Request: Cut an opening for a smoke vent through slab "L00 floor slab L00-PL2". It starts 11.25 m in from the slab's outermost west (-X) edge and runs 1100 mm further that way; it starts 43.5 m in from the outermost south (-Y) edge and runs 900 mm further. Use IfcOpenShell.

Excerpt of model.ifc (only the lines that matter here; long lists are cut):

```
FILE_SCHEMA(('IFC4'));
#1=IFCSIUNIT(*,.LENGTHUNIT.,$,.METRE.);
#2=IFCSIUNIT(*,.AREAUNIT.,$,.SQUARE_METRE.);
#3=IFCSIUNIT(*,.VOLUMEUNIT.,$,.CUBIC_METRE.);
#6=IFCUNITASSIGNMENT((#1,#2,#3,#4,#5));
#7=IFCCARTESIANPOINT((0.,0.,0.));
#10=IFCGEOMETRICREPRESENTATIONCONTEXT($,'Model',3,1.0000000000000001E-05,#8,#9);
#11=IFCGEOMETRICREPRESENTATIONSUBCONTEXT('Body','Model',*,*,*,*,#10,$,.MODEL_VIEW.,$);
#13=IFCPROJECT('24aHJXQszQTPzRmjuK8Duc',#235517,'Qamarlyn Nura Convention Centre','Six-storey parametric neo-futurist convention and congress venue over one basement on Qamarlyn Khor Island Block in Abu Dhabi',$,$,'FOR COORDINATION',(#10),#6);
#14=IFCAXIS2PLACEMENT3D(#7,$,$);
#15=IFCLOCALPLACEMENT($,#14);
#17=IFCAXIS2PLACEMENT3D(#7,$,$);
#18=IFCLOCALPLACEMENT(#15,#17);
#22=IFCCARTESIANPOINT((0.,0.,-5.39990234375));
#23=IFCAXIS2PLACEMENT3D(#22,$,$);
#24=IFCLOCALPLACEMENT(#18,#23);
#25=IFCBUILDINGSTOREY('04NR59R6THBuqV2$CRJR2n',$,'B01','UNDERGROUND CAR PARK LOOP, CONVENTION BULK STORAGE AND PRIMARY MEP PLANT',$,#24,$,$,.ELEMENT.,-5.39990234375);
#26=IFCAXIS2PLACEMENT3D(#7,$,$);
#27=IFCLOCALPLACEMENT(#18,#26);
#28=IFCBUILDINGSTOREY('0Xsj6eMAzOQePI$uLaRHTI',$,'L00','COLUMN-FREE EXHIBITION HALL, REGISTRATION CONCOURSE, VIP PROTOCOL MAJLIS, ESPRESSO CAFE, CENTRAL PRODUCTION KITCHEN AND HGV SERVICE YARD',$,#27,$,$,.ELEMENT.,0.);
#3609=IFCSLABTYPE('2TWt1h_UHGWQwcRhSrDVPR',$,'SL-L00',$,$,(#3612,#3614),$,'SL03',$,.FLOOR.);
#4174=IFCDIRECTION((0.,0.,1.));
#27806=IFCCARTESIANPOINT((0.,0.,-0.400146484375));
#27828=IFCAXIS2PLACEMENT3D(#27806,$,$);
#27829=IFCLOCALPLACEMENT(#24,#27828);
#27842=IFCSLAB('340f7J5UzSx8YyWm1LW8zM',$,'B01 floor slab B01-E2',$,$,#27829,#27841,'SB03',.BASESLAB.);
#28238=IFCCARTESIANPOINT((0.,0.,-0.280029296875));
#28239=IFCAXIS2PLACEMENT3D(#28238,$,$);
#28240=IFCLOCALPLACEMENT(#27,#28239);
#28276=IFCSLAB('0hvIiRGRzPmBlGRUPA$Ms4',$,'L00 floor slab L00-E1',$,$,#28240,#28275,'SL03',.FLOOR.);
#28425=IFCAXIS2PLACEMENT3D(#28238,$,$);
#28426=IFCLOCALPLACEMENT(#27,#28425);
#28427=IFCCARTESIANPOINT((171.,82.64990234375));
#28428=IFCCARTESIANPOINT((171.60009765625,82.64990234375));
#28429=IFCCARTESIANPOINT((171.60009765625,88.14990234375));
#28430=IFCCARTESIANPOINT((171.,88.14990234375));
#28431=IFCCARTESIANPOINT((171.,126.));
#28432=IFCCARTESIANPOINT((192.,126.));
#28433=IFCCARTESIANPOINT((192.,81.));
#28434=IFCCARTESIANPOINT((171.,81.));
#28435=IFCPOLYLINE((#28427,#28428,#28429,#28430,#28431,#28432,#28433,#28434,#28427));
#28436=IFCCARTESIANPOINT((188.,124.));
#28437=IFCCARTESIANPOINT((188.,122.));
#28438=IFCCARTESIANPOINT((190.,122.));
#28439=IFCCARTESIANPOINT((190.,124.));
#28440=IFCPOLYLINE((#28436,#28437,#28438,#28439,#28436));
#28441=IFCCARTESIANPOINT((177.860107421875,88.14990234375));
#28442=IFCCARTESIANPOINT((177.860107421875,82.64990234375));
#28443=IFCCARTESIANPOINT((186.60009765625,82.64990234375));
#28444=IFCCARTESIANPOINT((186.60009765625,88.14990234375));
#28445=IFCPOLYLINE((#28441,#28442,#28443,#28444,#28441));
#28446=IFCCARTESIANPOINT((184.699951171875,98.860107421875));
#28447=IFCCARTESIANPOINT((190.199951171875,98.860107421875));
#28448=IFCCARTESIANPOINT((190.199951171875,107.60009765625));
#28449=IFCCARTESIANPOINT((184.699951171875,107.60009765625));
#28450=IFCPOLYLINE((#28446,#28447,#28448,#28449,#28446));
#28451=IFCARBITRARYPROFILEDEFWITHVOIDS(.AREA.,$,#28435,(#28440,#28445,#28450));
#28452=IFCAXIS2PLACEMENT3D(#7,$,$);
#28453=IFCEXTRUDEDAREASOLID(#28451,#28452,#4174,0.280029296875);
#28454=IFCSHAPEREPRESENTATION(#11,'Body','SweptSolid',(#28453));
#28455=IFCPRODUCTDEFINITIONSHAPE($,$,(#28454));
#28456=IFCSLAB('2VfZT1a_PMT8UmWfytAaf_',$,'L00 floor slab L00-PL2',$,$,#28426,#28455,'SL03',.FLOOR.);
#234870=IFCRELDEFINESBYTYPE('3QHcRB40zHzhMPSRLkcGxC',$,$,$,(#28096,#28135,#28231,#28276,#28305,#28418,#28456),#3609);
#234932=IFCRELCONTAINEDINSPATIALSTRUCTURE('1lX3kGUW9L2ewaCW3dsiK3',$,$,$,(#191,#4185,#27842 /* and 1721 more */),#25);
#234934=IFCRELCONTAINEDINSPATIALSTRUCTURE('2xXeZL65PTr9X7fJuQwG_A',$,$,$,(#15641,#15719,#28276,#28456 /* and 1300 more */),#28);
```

```python
import numpy as np
import ifcopenshell
import ifcopenshell.api.feature
import ifcopenshell.api.geometry
import ifcopenshell.api.root
import ifcopenshell.geom
import ifcopenshell.util.placement
import ifcopenshell.util.representation
import ifcopenshell.util.shape
import ifcopenshell.util.unit

model = ifcopenshell.open("model.ifc")
unit_scale = ifcopenshell.util.unit.calculate_unit_scale(model)
settings = ifcopenshell.geom.settings()


def volume(element):
    """Net volume in cubic metres, openings subtracted."""
    shape = ifcopenshell.geom.create_shape(settings, element)
    return ifcopenshell.util.shape.get_volume(shape.geometry)


slab = model.by_guid("2VfZT1a_PMT8UmWfytAaf_")
before = volume(slab)

# Extent in the slab's own axes, in metres. The edges named are its -X and -Y sides.
slab_shape = ifcopenshell.geom.create_shape(settings, slab)
vertices = ifcopenshell.util.shape.get_vertices(slab_shape.geometry)
x_min, y_min, bottom = vertices.min(axis=0)
top = vertices[:, 2].max()

opening = ifcopenshell.api.root.create_entity(model, ifc_class="IfcOpeningElement", name="Smoke vent opening", predefined_type="OPENING")
context = ifcopenshell.util.representation.get_context(model, "Model", "Body", "MODEL_VIEW")
width, depth = 1.1, 0.9
outline = [(0.0, 0.0), (width, 0.0), (width, depth), (0.0, depth), (0.0, 0.0)]
# Overshoot both faces by 50 mm so the cut is clean.
shape = ifcopenshell.api.geometry.add_slab_representation(
    model, context=context, depth=top - bottom + 0.1, polyline=outline
)
ifcopenshell.api.geometry.assign_representation(model, product=opening, representation=shape)

matrix = ifcopenshell.util.placement.get_local_placement(slab.ObjectPlacement)
matrix[:, 3] = matrix @ np.append(np.array([x_min + 11.25, y_min + 43.5, bottom - 0.05]) / unit_scale, 1.0)
ifcopenshell.api.geometry.edit_object_placement(model, product=opening, matrix=matrix, is_si=False)
ifcopenshell.api.feature.add_feature(model, feature=opening, element=slab)

after = volume(slab)

print(f"slab volume {before:.3f} -> {after:.3f} m3")

model.write("model-out.ifc")
```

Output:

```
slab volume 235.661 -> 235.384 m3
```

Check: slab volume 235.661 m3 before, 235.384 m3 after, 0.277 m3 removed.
